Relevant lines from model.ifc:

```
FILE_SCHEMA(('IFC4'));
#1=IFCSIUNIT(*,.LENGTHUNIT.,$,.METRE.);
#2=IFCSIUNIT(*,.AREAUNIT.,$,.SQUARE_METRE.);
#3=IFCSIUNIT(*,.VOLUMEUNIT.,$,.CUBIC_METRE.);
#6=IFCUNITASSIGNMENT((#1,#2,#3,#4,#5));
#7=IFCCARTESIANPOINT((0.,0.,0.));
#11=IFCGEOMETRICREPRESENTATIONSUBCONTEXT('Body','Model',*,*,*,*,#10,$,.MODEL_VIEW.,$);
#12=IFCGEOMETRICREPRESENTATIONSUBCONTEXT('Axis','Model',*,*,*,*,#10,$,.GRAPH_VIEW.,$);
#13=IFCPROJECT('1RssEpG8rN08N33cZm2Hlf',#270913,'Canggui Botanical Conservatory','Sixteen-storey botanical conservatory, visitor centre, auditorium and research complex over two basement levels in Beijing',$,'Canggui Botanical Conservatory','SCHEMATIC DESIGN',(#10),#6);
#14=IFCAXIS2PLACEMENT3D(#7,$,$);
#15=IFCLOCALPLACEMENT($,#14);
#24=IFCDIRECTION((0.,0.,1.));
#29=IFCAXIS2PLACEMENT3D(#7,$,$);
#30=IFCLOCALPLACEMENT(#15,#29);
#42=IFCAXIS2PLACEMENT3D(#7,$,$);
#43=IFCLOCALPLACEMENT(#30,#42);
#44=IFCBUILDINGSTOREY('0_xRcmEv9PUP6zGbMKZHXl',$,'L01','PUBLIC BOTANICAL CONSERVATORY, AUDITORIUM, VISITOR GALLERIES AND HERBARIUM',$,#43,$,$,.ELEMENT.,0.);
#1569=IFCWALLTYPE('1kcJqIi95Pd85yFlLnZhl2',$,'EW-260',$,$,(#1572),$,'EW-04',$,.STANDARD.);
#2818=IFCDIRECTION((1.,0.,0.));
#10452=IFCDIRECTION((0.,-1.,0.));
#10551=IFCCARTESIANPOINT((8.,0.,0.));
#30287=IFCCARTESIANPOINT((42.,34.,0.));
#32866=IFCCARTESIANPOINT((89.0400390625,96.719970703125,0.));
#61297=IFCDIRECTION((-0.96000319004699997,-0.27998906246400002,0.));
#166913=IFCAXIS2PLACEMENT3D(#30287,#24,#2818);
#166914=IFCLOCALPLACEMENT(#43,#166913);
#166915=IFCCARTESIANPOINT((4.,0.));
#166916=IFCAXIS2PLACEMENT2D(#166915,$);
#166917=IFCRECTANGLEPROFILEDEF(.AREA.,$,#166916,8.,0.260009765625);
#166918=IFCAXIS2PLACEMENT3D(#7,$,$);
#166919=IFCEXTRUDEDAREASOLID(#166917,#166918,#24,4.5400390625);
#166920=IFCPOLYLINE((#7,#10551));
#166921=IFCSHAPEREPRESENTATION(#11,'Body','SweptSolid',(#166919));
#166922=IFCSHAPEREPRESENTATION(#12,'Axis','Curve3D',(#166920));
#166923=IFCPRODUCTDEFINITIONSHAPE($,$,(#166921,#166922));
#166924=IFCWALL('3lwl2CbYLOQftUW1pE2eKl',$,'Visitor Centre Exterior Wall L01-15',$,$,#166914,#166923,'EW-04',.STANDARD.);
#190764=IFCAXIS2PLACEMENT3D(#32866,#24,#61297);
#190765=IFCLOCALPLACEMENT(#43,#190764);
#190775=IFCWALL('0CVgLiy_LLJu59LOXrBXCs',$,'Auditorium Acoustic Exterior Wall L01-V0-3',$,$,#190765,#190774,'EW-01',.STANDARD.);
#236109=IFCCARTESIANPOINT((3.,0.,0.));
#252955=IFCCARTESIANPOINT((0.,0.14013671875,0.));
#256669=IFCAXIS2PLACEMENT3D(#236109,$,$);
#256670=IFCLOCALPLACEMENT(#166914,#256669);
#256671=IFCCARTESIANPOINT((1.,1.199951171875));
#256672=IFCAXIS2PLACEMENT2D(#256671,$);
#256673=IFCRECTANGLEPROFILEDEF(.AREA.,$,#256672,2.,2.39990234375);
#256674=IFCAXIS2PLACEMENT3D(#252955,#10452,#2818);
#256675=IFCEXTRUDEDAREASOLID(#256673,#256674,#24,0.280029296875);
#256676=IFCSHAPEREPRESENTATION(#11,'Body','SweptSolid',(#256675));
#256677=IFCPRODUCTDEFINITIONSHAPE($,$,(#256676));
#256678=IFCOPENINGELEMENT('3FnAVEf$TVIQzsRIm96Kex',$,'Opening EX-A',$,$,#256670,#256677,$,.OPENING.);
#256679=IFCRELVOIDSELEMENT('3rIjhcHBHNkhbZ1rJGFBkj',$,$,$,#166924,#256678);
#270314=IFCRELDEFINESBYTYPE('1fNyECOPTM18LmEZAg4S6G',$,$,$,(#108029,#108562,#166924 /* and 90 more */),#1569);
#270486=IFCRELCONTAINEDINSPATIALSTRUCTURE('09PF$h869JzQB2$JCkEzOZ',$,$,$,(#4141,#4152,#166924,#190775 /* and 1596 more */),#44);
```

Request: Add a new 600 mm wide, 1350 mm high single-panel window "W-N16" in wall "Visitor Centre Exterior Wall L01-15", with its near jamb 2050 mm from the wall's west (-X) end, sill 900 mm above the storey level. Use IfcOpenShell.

```python
import numpy as np
import ifcopenshell
import ifcopenshell.api.feature
import ifcopenshell.api.geometry
import ifcopenshell.api.root
import ifcopenshell.api.spatial
import ifcopenshell.geom
import ifcopenshell.util.element
import ifcopenshell.util.placement
import ifcopenshell.util.representation
import ifcopenshell.util.shape
import ifcopenshell.util.unit

model = ifcopenshell.open("model.ifc")
unit_scale = ifcopenshell.util.unit.calculate_unit_scale(model)
settings = ifcopenshell.geom.settings()


def volume(element):
    """Net volume in cubic metres, openings subtracted."""
    shape = ifcopenshell.geom.create_shape(settings, element)
    return ifcopenshell.util.shape.get_volume(shape.geometry)


wall = model.by_guid("3lwl2CbYLOQftUW1pE2eKl")
storey = ifcopenshell.util.element.get_container(wall, ifc_class="IfcBuildingStorey")
context = ifcopenshell.util.representation.get_context(model, "Model", "Body", "MODEL_VIEW")
before = volume(wall)

width, height, from_end, sill = 0.6, 1.35, 2.05, 0.9  # metres

# The wall runs along its own X axis, and the end named is its -X end.
wall_shape = ifcopenshell.geom.create_shape(settings, wall)
x, y, z = ifcopenshell.util.shape.get_vertices(wall_shape.geometry).T
start = x.min() + from_end
face, thickness = float(y.min()), float(y.max() - y.min())
wall_matrix = ifcopenshell.util.placement.get_local_placement(wall.ObjectPlacement)
level = ifcopenshell.util.placement.get_local_placement(storey.ObjectPlacement)[2, 3]


def in_wall(x, y):
    """Placement at x, y metres in the wall's axes, at sill height."""
    matrix = wall_matrix.copy()
    matrix[:, 3] = wall_matrix @ np.array([x / unit_scale, y / unit_scale, 0.0, 1.0])
    matrix[2, 3] = level + sill / unit_scale
    return matrix


# Opening: a box that overshoots both wall faces by 50 mm.
opening = ifcopenshell.api.root.create_entity(model, ifc_class="IfcOpeningElement", predefined_type="OPENING")
box = ifcopenshell.api.geometry.add_wall_representation(
    model, context=context, length=width, height=height, thickness=thickness + 0.1
)
ifcopenshell.api.geometry.assign_representation(model, product=opening, representation=box)
ifcopenshell.api.geometry.edit_object_placement(model, product=opening, matrix=in_wall(start, face - 0.05), is_si=False)
ifcopenshell.api.feature.add_feature(model, feature=opening, element=wall)

window = ifcopenshell.api.root.create_entity(model, ifc_class="IfcWindow", name="W-N16", predefined_type="WINDOW")
window.OverallWidth, window.OverallHeight = width / unit_scale, height / unit_scale
window.PartitioningType = "SINGLE_PANEL"
body = ifcopenshell.api.geometry.add_window_representation(
    model,
    context=context,
    overall_width=window.OverallWidth,
    overall_height=window.OverallHeight,
    partition_type="SINGLE_PANEL",
)
ifcopenshell.api.geometry.assign_representation(model, product=window, representation=body)
ifcopenshell.api.spatial.assign_container(model, products=[window], relating_structure=storey)
ifcopenshell.api.feature.add_filling(model, opening=opening, element=window)

# Centre the window in the wall's thickness.
ifcopenshell.api.geometry.edit_object_placement(model, product=window, matrix=in_wall(start, face), is_si=False)
window_shape = ifcopenshell.geom.create_shape(settings, window)
depth = ifcopenshell.util.shape.get_vertices(window_shape.geometry)[:, 1]
offset = face + thickness / 2 - (depth.min() + depth.max()) / 2
ifcopenshell.api.geometry.edit_object_placement(model, product=window, matrix=in_wall(start, offset), is_si=False)

after = volume(wall)

print(f"wall volume {before:.3f} -> {after:.3f} m3")

model.write("model_v2.ifc")
```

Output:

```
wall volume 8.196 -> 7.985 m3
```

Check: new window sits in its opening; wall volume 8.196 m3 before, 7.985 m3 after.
